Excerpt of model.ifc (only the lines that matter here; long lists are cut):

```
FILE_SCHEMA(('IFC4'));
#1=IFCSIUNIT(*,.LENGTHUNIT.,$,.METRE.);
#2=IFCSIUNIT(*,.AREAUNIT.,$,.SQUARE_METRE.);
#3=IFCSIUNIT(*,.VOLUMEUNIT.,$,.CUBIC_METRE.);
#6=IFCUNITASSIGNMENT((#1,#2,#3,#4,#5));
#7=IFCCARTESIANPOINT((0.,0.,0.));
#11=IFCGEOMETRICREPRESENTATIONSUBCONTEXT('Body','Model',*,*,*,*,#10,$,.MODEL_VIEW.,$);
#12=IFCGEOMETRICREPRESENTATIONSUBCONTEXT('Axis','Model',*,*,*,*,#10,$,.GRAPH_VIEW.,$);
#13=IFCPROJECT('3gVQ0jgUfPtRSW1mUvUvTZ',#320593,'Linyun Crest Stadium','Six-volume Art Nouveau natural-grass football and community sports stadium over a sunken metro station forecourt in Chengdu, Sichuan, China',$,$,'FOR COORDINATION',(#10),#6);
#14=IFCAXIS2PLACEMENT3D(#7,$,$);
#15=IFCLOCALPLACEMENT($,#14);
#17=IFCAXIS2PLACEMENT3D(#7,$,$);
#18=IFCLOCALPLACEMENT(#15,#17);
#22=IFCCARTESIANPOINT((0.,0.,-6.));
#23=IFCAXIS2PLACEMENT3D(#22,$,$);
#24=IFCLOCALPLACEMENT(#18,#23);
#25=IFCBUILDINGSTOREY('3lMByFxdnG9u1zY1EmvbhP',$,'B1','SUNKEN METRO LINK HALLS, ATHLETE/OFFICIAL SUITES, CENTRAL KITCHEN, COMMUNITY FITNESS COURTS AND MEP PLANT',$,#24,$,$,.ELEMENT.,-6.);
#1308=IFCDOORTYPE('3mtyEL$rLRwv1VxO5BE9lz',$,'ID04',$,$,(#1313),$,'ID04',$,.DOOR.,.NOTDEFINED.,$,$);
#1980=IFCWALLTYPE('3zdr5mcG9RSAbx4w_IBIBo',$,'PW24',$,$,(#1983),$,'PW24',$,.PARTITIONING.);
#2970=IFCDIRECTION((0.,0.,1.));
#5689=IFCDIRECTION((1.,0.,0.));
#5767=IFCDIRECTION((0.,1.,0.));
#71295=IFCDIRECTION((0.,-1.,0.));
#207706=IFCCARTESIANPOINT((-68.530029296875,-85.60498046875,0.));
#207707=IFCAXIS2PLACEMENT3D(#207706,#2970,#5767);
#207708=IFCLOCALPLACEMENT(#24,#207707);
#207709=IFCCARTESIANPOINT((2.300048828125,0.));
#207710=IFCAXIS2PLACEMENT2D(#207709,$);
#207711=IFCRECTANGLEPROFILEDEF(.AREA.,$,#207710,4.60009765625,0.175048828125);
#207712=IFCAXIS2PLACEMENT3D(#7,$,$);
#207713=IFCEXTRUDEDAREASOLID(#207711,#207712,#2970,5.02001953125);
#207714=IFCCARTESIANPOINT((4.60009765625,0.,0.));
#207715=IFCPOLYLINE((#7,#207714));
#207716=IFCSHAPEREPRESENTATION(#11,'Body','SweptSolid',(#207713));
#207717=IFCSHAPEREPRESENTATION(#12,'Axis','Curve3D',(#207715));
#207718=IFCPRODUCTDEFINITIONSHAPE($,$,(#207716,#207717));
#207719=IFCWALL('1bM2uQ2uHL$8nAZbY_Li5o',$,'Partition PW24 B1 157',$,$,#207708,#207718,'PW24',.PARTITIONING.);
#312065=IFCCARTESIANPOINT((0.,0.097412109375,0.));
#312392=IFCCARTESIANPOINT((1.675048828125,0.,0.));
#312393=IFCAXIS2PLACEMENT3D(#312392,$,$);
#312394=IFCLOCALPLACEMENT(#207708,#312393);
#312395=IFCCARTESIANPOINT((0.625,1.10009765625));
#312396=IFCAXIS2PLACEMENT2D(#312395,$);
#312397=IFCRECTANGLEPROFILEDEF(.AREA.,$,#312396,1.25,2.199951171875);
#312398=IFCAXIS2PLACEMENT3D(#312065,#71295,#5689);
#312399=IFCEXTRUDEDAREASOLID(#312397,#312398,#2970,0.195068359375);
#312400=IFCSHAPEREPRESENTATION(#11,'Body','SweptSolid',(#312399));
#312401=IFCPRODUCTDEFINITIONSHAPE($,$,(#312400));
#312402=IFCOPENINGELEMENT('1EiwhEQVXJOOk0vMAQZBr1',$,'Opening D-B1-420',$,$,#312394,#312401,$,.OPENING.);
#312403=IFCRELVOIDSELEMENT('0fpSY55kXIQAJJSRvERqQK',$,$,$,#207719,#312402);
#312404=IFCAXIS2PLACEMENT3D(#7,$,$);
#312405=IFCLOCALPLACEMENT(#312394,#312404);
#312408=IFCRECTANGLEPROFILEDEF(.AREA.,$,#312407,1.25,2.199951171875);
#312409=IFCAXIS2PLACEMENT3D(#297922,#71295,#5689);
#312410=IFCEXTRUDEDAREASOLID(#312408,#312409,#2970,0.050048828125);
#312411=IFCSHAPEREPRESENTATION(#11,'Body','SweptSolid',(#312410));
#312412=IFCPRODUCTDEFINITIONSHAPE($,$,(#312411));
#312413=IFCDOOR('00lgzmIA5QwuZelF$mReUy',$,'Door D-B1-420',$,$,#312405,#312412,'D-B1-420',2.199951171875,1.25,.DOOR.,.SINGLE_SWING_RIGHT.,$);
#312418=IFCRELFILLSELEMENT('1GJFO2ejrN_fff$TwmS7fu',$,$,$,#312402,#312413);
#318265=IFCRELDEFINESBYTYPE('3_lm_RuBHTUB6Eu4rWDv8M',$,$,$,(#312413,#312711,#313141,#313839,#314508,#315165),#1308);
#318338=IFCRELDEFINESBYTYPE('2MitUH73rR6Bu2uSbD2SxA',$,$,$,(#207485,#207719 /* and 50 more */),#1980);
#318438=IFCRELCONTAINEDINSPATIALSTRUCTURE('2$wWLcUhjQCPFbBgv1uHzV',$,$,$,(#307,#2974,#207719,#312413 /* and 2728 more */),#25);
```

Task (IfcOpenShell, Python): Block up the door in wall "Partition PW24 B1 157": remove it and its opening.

```python
import ifcopenshell
import ifcopenshell.api.feature
import ifcopenshell.api.root
import ifcopenshell.geom
import ifcopenshell.util.shape

model = ifcopenshell.open("model.ifc")
settings = ifcopenshell.geom.settings()


def volume(element):
    """Net volume in cubic metres, openings subtracted."""
    shape = ifcopenshell.geom.create_shape(settings, element)
    return ifcopenshell.util.shape.get_volume(shape.geometry)


door = model.by_id(312413)
opening = door.FillsVoids[0].RelatingOpeningElement
wall = opening.VoidsElements[0].RelatingBuildingElement
before = volume(wall)

ifcopenshell.api.root.remove_product(model, product=door)
ifcopenshell.api.feature.remove_feature(model, feature=opening)

after = volume(wall)

print(f"wall volume {before:.3f} -> {after:.3f} m3")

model.write("model-out.ifc")
```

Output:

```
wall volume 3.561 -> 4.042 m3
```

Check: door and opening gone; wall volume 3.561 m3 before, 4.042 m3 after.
